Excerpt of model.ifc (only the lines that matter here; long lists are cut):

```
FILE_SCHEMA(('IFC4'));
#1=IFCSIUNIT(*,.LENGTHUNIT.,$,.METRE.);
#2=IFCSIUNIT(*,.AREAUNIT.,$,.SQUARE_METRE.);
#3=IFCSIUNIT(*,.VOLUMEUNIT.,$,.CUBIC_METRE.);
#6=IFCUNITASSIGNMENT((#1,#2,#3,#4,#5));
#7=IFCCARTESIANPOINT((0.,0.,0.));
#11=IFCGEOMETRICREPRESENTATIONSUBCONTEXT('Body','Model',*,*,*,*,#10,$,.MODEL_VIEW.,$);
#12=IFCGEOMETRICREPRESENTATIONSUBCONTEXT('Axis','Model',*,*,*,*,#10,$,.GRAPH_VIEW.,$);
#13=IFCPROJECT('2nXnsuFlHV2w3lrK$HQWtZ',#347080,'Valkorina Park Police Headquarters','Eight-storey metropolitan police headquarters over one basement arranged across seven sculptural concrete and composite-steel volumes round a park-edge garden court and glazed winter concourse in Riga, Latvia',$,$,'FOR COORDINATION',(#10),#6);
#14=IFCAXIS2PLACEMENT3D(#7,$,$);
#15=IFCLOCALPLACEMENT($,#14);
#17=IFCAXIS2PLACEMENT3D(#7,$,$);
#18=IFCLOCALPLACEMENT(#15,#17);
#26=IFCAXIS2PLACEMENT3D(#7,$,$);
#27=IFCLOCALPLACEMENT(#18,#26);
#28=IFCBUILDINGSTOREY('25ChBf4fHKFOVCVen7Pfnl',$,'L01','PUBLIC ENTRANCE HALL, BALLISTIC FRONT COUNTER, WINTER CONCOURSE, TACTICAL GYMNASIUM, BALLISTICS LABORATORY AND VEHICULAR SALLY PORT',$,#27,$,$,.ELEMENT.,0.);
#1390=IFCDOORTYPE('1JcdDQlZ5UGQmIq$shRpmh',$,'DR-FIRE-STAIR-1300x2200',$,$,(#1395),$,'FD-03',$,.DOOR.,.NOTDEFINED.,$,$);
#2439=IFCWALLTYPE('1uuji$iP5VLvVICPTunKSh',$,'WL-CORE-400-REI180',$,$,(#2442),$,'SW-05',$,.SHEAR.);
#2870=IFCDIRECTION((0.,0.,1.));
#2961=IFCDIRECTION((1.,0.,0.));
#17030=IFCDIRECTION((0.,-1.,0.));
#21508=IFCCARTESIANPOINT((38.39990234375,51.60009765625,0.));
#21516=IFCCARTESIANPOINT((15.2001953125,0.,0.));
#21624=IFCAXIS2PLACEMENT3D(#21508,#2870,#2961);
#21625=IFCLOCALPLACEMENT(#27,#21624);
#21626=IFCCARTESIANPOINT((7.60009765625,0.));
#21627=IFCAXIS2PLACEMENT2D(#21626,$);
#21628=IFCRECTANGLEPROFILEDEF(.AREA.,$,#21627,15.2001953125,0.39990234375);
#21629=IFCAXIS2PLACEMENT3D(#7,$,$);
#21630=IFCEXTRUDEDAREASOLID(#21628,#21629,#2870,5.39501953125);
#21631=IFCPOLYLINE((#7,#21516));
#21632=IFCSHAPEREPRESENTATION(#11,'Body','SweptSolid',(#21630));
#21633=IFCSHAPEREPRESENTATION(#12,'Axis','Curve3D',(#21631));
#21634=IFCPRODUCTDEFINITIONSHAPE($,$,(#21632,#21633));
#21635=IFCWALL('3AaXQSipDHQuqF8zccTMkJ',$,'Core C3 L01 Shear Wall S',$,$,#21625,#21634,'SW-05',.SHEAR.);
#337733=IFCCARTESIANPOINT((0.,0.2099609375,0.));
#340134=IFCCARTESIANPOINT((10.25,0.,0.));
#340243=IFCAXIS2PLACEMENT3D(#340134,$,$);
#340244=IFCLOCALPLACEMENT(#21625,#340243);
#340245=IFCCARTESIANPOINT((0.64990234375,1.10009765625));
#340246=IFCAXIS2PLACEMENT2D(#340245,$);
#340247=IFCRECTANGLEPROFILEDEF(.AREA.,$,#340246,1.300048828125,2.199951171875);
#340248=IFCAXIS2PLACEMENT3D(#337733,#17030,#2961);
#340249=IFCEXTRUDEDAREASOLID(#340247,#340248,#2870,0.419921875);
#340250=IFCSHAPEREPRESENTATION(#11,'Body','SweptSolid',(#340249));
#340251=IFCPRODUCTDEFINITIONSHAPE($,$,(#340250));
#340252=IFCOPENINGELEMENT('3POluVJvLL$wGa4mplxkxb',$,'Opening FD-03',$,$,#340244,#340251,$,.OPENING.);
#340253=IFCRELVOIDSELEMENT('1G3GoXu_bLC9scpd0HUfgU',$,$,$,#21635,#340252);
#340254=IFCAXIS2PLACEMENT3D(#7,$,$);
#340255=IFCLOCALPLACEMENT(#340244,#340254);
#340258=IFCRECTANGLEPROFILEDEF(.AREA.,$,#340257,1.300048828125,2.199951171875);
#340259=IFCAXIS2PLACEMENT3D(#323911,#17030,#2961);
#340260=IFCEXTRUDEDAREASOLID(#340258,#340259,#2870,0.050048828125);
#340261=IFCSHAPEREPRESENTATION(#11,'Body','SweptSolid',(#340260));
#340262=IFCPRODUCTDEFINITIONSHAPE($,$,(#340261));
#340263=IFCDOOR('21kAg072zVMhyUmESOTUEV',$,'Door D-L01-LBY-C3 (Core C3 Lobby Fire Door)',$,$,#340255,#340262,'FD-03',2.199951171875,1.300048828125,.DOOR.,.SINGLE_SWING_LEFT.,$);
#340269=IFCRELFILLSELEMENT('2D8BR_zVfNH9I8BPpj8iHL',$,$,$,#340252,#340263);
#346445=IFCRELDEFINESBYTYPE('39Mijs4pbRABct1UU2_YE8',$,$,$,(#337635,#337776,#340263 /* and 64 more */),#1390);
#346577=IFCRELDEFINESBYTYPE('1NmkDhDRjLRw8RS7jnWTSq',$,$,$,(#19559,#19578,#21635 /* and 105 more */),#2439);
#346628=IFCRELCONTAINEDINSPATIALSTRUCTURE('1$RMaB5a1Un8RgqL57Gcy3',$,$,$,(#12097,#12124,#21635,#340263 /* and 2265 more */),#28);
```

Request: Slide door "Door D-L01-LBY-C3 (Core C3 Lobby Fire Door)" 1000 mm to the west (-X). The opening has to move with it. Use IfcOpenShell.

```python
import ifcopenshell
import ifcopenshell.api.geometry
import ifcopenshell.util.placement

model = ifcopenshell.open("model.ifc")

door = model.by_guid("21kAg072zVMhyUmESOTUEV")
opening = door.FillsVoids[0].RelatingOpeningElement
wall = opening.VoidsElements[0].RelatingBuildingElement

wall_matrix = ifcopenshell.util.placement.get_local_placement(wall.ObjectPlacement)
shift = wall_matrix[:3, 0] * -1.0
before = ifcopenshell.util.placement.get_local_placement(door.ObjectPlacement)[:3, 3].copy()

# The door is placed relative to its opening, so it follows when the opening moves.
matrix = ifcopenshell.util.placement.get_local_placement(opening.ObjectPlacement)
matrix[:3, 3] += shift
ifcopenshell.api.geometry.edit_object_placement(
    model, product=opening, matrix=matrix, is_si=False, should_transform_children=True
)

after = ifcopenshell.util.placement.get_local_placement(door.ObjectPlacement)[:3, 3]
print("door moved by", (after - before).round(3) + 0.0)

model.write("model_v2.ifc")
```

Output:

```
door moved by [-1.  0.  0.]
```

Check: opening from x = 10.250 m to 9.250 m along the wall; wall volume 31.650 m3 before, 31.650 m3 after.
